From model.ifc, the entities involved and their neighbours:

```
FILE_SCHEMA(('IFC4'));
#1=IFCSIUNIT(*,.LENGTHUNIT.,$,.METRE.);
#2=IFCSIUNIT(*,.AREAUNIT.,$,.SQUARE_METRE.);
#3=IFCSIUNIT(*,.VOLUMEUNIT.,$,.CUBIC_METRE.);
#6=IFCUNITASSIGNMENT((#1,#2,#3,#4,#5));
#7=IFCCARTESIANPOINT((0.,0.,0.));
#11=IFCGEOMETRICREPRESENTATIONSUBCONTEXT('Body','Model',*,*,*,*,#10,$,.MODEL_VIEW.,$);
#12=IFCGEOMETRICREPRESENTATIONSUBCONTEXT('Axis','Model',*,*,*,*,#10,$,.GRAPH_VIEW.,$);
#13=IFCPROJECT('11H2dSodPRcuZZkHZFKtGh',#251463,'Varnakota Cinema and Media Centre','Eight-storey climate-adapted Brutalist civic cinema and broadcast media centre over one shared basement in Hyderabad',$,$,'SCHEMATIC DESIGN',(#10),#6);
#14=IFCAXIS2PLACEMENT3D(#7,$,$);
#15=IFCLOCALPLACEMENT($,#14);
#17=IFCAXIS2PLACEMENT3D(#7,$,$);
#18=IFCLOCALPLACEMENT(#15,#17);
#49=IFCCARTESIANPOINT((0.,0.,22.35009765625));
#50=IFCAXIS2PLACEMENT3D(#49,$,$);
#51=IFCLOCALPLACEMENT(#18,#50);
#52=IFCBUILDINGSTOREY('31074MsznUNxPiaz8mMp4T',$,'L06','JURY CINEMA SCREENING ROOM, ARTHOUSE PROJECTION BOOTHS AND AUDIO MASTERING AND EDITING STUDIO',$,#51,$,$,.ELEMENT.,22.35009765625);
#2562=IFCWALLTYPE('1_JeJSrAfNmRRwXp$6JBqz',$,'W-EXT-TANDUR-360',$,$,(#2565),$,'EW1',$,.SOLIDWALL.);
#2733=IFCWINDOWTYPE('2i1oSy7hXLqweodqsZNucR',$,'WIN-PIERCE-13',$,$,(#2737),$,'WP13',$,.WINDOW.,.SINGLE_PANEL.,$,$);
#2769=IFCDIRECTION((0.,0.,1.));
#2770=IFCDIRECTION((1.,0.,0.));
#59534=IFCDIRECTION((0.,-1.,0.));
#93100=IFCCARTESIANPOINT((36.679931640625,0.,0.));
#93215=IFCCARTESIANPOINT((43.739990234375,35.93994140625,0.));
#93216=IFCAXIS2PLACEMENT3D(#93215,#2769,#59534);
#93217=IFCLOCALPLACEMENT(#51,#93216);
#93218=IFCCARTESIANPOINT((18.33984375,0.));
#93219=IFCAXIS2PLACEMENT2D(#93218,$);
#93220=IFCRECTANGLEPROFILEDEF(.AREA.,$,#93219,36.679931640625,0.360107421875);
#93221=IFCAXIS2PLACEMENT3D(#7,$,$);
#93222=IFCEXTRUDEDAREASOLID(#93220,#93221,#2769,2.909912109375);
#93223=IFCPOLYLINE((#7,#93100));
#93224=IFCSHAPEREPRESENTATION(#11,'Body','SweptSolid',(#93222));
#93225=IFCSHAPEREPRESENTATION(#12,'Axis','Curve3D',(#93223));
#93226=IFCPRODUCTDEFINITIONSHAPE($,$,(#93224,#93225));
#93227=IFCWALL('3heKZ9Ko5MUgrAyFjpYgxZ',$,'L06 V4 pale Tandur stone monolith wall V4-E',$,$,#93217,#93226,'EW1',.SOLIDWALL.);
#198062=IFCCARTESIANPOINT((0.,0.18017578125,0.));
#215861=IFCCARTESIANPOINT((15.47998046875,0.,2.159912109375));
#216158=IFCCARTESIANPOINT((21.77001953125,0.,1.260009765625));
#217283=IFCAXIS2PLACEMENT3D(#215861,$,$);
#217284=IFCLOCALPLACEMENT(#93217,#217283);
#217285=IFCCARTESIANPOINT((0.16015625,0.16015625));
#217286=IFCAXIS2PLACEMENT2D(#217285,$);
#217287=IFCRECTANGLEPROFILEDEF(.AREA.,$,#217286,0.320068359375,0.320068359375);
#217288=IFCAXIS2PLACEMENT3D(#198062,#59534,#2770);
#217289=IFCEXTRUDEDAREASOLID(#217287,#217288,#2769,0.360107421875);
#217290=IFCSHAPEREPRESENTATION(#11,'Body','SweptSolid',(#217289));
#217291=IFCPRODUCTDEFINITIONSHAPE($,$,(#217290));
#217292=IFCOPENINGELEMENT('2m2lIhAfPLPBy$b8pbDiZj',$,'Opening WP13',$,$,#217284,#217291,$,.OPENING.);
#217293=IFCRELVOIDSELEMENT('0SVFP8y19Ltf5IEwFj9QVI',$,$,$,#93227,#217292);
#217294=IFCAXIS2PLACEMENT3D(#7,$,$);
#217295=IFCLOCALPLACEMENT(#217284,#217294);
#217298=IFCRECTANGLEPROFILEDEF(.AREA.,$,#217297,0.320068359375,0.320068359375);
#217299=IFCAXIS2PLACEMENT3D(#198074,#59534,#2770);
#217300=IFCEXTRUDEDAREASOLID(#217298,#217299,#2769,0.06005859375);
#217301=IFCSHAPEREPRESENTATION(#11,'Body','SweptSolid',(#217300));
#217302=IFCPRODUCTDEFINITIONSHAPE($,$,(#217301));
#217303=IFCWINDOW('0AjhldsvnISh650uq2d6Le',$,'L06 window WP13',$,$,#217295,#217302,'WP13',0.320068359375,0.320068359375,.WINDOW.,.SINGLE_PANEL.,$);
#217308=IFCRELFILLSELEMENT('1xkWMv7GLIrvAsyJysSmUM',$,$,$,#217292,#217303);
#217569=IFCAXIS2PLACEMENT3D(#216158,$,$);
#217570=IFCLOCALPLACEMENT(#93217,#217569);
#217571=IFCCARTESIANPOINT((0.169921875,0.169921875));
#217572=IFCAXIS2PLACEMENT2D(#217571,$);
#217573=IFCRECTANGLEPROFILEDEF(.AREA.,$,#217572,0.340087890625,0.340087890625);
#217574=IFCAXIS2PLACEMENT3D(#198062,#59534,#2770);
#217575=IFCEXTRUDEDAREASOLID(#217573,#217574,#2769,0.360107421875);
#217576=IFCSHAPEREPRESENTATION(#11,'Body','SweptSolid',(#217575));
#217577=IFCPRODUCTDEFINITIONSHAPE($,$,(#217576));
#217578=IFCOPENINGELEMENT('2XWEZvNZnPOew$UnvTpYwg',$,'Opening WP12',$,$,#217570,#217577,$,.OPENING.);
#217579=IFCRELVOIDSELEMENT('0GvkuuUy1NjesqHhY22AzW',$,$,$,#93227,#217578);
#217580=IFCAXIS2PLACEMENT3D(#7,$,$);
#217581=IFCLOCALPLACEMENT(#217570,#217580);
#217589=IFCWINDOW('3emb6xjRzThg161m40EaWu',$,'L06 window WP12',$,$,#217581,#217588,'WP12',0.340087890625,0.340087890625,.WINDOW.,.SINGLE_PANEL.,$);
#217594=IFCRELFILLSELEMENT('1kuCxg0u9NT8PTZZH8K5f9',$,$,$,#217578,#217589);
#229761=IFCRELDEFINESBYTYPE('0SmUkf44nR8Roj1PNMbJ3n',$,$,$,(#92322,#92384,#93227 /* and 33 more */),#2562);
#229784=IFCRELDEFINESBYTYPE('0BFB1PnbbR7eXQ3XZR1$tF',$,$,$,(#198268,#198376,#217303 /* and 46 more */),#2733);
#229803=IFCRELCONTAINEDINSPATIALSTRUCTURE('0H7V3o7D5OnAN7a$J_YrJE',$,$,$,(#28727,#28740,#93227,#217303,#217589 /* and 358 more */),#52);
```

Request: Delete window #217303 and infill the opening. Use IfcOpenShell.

```python
import ifcopenshell
import ifcopenshell.api.feature
import ifcopenshell.api.root
import ifcopenshell.geom
import ifcopenshell.util.shape

model = ifcopenshell.open("model.ifc")
settings = ifcopenshell.geom.settings()


def volume(element):
    """Net volume in cubic metres, openings subtracted."""
    shape = ifcopenshell.geom.create_shape(settings, element)
    return ifcopenshell.util.shape.get_volume(shape.geometry)


window = model.by_id(217303)
opening = window.FillsVoids[0].RelatingOpeningElement
wall = opening.VoidsElements[0].RelatingBuildingElement
before = volume(wall)

ifcopenshell.api.root.remove_product(model, product=window)
ifcopenshell.api.feature.remove_feature(model, feature=opening)

after = volume(wall)

print(f"wall volume {before:.3f} -> {after:.3f} m3")

model.write("model_updated.ifc")
```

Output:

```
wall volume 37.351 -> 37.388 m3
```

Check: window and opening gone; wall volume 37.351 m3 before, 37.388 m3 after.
